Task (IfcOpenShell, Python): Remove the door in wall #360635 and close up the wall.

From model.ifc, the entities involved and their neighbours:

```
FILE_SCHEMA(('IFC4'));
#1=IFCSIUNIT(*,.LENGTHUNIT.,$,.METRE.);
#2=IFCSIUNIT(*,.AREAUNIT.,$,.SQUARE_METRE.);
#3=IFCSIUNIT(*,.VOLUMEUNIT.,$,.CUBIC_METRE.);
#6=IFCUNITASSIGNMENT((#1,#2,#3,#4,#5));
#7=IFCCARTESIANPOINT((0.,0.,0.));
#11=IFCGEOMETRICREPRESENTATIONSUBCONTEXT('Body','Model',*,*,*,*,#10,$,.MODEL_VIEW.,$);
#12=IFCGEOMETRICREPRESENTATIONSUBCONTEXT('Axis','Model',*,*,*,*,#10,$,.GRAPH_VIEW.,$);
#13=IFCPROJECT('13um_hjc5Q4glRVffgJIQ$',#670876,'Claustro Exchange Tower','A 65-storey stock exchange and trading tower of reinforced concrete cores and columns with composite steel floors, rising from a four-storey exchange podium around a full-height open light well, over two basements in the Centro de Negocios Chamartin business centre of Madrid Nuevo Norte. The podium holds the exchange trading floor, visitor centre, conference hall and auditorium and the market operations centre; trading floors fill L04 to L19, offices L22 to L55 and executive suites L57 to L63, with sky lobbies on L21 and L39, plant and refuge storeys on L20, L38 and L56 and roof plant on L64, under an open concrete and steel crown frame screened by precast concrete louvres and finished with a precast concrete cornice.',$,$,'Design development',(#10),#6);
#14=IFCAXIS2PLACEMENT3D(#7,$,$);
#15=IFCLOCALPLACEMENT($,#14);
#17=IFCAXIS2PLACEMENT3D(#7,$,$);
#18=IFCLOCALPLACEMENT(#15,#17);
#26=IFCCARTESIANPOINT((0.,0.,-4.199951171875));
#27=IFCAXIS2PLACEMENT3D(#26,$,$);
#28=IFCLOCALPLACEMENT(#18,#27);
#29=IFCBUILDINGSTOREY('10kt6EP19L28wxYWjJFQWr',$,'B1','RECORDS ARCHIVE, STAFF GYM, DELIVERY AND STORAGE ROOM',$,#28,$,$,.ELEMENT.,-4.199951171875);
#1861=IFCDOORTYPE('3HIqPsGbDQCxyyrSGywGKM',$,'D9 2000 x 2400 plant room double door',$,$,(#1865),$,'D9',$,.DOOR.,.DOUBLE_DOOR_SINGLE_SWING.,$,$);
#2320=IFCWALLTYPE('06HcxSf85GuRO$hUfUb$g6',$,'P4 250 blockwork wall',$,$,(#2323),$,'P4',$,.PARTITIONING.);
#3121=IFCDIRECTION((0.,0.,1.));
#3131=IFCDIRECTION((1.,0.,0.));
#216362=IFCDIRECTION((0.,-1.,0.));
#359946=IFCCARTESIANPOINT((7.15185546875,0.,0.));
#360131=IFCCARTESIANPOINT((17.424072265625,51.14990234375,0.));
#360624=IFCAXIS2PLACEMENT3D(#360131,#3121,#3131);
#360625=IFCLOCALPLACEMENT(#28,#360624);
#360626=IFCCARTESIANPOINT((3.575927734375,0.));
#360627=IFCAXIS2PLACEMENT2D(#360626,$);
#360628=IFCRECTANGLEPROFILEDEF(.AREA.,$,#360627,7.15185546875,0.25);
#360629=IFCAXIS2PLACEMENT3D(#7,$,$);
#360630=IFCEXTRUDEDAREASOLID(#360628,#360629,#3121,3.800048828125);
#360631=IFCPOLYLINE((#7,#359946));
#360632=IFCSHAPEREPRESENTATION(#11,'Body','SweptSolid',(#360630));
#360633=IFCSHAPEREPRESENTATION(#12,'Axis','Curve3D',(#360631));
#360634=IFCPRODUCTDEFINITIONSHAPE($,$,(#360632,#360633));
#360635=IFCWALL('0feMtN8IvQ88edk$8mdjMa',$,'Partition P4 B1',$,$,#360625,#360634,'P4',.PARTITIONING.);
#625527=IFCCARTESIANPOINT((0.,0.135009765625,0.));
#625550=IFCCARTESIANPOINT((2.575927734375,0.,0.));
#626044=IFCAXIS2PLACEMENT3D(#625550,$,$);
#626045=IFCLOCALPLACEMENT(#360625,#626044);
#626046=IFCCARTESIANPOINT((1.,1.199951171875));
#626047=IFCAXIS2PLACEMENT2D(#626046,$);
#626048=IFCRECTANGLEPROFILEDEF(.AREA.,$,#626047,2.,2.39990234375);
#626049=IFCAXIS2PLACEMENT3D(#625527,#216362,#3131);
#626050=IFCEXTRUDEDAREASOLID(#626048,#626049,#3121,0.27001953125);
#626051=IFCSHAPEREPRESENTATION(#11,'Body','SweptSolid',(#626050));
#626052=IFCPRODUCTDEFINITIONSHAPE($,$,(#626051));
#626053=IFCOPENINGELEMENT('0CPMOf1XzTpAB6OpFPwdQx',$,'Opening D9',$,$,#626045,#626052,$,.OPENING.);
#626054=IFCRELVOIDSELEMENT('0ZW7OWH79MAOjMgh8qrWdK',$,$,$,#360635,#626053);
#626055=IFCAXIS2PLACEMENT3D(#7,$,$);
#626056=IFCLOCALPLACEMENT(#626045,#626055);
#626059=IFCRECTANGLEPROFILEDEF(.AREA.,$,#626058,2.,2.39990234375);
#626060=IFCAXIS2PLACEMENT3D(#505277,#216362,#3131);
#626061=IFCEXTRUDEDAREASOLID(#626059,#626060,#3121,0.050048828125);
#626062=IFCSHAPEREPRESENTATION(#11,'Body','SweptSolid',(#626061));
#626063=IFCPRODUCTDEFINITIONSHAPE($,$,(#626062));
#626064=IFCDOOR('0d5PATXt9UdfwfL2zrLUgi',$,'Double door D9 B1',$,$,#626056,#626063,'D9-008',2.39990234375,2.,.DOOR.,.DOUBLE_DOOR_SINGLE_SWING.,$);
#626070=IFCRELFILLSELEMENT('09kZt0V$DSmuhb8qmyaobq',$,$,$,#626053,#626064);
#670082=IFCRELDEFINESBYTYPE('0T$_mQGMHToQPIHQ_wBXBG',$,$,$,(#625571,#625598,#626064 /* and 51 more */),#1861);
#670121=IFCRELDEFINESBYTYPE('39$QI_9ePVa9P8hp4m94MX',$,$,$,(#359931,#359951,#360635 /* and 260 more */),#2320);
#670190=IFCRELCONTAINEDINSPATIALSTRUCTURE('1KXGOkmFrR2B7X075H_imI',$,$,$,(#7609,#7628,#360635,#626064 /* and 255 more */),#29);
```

```python
import ifcopenshell
import ifcopenshell.api.feature
import ifcopenshell.api.root
import ifcopenshell.geom
import ifcopenshell.util.shape

model = ifcopenshell.open("model.ifc")
settings = ifcopenshell.geom.settings()


def volume(element):
    """Net volume in cubic metres, openings subtracted."""
    shape = ifcopenshell.geom.create_shape(settings, element)
    return ifcopenshell.util.shape.get_volume(shape.geometry)


door = model.by_id(626064)
opening = door.FillsVoids[0].RelatingOpeningElement
wall = opening.VoidsElements[0].RelatingBuildingElement
before = volume(wall)

ifcopenshell.api.root.remove_product(model, product=door)
ifcopenshell.api.feature.remove_feature(model, feature=opening)

after = volume(wall)

print(f"wall volume {before:.3f} -> {after:.3f} m3")

model.write("model-out.ifc")
```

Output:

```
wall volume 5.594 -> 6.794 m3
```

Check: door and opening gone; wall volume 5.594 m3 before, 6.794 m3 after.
